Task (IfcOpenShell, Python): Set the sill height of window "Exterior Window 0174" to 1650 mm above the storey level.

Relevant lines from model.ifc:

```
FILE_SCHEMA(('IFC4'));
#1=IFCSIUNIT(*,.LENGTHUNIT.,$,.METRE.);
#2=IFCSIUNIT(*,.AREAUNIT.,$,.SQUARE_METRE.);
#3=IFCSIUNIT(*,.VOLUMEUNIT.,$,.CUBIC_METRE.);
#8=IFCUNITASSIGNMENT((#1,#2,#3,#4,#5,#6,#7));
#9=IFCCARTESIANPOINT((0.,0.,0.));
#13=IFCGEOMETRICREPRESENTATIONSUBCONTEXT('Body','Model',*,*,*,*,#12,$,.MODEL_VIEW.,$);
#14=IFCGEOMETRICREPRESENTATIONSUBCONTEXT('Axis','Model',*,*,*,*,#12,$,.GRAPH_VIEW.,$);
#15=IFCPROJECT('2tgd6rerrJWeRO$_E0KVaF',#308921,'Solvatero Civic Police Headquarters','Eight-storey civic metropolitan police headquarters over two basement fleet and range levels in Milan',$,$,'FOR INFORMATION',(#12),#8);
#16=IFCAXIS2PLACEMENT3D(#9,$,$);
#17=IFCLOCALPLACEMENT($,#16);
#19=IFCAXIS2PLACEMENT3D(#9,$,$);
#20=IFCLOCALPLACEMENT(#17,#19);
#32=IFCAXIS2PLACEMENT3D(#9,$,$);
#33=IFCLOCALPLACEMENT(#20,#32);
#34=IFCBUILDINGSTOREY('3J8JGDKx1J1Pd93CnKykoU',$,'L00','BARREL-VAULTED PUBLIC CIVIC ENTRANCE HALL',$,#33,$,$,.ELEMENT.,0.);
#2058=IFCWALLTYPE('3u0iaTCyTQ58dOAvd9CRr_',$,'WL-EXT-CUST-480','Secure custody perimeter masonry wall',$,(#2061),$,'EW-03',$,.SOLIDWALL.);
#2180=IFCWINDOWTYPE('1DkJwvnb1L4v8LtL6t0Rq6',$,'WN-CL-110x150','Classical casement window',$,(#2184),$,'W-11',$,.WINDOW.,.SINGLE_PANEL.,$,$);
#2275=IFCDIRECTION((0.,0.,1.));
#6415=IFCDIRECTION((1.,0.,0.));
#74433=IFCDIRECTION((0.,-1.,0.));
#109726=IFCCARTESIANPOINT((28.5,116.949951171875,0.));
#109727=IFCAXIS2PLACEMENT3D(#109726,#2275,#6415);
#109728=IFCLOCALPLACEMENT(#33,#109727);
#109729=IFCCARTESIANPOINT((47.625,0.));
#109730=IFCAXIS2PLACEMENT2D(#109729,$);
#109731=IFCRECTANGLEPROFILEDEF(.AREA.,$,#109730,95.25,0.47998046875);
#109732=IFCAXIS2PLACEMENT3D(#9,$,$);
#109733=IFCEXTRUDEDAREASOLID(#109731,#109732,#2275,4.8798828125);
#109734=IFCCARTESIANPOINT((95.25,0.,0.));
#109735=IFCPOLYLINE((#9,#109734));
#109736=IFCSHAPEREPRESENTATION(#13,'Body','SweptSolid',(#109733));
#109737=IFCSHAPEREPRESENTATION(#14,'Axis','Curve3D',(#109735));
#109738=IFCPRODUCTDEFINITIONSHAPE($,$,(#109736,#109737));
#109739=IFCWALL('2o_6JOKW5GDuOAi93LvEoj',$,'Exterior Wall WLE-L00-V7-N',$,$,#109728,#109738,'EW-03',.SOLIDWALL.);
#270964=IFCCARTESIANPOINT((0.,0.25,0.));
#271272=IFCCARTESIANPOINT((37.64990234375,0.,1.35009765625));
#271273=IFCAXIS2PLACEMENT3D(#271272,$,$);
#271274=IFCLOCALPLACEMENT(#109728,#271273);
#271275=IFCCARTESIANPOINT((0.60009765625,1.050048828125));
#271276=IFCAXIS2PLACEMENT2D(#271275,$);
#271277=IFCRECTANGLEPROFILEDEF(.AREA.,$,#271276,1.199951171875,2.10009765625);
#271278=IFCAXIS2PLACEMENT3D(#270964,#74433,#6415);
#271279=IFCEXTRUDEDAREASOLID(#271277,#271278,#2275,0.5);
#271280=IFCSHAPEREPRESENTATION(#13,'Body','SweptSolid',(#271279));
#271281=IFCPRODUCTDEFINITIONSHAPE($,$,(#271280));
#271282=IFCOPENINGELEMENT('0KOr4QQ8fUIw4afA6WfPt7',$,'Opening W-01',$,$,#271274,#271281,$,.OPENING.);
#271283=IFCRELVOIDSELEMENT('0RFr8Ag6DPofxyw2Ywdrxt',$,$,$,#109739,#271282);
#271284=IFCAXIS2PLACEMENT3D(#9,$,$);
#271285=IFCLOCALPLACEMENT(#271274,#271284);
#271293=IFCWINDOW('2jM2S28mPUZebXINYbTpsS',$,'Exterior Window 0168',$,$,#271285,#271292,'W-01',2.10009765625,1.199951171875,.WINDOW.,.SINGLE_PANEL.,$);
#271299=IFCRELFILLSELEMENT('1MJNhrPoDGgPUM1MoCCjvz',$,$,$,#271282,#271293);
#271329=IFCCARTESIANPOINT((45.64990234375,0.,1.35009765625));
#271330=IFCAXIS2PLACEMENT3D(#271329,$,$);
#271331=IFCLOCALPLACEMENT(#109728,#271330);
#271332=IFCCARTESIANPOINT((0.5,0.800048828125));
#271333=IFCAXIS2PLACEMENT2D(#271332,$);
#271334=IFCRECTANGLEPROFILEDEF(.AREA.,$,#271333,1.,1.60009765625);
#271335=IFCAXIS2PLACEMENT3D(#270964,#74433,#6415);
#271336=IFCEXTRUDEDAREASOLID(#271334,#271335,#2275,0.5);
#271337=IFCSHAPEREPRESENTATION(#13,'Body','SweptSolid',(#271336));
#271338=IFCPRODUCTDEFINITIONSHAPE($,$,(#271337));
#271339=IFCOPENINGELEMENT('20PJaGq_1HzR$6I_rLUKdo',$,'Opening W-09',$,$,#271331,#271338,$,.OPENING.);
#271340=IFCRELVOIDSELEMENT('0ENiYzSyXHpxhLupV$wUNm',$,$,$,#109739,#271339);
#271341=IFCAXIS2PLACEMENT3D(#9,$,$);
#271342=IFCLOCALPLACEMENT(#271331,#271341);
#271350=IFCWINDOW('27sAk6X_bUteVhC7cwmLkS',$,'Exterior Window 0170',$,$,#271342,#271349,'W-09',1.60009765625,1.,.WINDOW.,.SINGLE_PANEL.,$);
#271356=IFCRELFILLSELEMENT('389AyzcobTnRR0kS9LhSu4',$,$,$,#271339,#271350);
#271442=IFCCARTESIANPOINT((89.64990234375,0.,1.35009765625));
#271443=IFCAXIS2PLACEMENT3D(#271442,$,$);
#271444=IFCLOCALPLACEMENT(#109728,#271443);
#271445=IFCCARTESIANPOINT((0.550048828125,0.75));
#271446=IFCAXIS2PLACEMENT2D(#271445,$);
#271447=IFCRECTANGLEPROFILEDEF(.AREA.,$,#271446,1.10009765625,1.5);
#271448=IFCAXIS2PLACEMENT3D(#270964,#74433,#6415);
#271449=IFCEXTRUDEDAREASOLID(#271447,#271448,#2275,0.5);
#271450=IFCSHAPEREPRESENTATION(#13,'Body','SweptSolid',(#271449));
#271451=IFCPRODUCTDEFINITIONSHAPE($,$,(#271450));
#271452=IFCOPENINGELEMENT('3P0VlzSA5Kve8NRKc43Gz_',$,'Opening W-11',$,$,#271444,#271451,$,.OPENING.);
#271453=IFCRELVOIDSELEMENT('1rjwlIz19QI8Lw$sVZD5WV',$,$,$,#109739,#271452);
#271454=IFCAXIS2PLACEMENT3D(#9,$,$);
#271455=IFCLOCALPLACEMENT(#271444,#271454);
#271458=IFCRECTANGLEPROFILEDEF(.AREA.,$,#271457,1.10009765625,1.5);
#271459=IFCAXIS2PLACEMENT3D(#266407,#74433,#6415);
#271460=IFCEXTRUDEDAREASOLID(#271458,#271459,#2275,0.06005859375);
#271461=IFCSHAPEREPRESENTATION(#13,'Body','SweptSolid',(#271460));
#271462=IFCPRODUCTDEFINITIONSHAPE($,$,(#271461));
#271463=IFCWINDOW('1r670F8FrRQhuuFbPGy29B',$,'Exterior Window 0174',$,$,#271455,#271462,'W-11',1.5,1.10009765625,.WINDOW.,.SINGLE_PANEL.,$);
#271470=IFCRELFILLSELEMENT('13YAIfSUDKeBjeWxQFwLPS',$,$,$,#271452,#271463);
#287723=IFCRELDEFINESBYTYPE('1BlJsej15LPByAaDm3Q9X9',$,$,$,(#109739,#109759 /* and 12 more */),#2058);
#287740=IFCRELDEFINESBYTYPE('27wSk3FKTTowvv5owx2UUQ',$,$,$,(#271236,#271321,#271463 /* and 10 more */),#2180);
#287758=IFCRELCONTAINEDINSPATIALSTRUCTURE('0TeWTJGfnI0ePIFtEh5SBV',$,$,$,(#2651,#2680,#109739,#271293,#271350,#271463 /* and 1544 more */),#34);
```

```python
import numpy as np
import ifcopenshell
import ifcopenshell.api.geometry
import ifcopenshell.geom
import ifcopenshell.util.element
import ifcopenshell.util.placement
import ifcopenshell.util.shape
import ifcopenshell.util.unit

model = ifcopenshell.open("model.ifc")
unit_scale = ifcopenshell.util.unit.calculate_unit_scale(model)

window = model.by_guid("1r670F8FrRQhuuFbPGy29B")
opening = window.FillsVoids[0].RelatingOpeningElement
storey = ifcopenshell.util.element.get_container(window, ifc_class="IfcBuildingStorey")
level = ifcopenshell.util.placement.get_local_placement(storey.ObjectPlacement)[2, 3]

# The opening's origin need not be at the sill, so measure its lowest point.
shape = ifcopenshell.geom.create_shape(ifcopenshell.geom.settings(), opening)
bottom = ifcopenshell.util.shape.get_shape_bottom_elevation(shape, shape.geometry) / unit_scale
dz = level + 1.65 / unit_scale - bottom

shift = np.array([0.0, 0.0, dz])
# The window is placed relative to its opening, so it follows when the opening moves.
matrix = ifcopenshell.util.placement.get_local_placement(opening.ObjectPlacement)
matrix[:3, 3] += shift
ifcopenshell.api.geometry.edit_object_placement(
    model, product=opening, matrix=matrix, is_si=False, should_transform_children=True
)

print(f"moved by {dz * unit_scale:+.3f} m")

model.write("model_rev.ifc")
```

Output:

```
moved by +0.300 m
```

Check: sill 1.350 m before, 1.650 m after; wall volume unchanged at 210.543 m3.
